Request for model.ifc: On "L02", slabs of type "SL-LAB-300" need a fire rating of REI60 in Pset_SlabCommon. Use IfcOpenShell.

First a look at what the model holds.

```python
import ifcopenshell
import ifcopenshell.util.element

model = ifcopenshell.open("model.ifc")
print(model.schema)
storey = next(s for s in model.by_type("IfcBuildingStorey") if s.Name == "L02")
slabs = [e for e in ifcopenshell.util.element.get_decomposition(storey) if e.is_a("IfcSlab")]
seen = {}
for e in slabs:
    element_type = ifcopenshell.util.element.get_type(e)
    key = (element_type.Name if element_type != e and element_type else None, ifcopenshell.util.element.get_pset(e, "Pset_SlabCommon", "FireRating"))
    seen[key] = seen.get(key, 0) + 1
for (name, value), count in sorted(seen.items(), key=str):
    print(count, "x", name, "|", value)
```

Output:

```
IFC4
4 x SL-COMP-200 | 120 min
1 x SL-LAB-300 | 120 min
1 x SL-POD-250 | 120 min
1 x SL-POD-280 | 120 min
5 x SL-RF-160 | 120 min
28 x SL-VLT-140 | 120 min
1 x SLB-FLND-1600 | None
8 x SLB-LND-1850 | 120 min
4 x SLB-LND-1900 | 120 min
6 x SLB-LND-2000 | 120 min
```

```python
import ifcopenshell
import ifcopenshell.api.pset
import ifcopenshell.util.element

model = ifcopenshell.open("model.ifc")

storey = next(s for s in model.by_type("IfcBuildingStorey") if s.Name == "L02")
slabs = [e for e in ifcopenshell.util.element.get_decomposition(storey) if e.is_a("IfcSlab")]

count = 0
for e in slabs:
    element_type = ifcopenshell.util.element.get_type(e)
    if element_type in (None, e) or element_type.Name != "SL-LAB-300":
        continue
    # add_pset returns the element's existing set when there is one.
    pset = ifcopenshell.api.pset.add_pset(model, product=e, name="Pset_SlabCommon")
    ifcopenshell.api.pset.edit_pset(model, pset=pset, properties={"FireRating": "REI60"})
    count += 1

print(count, "slabs updated")

model.write("model_updated.ifc")
```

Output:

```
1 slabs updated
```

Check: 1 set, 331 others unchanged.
